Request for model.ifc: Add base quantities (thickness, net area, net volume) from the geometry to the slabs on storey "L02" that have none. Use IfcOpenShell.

First a look at what the model holds.

```python
import ifcopenshell
import ifcopenshell.util.element
import ifcopenshell.util.unit

model = ifcopenshell.open("model.ifc")
print(model.schema)
for unit_type in ("LENGTHUNIT", "AREAUNIT", "VOLUMEUNIT"):
    print(unit_type, ifcopenshell.util.unit.calculate_unit_scale(model, unit_type))
storey = next(s for s in model.by_type("IfcBuildingStorey") if s.Name == "L02")
slabs = [e for e in ifcopenshell.util.element.get_decomposition(storey) if e.is_a("IfcSlab")]
for e in sorted(slabs, key=lambda e: e.id()):
    print(e.id(), e.is_a(), e.Name, list(ifcopenshell.util.element.get_psets(e, qtos_only=True)), sep=" | ")
```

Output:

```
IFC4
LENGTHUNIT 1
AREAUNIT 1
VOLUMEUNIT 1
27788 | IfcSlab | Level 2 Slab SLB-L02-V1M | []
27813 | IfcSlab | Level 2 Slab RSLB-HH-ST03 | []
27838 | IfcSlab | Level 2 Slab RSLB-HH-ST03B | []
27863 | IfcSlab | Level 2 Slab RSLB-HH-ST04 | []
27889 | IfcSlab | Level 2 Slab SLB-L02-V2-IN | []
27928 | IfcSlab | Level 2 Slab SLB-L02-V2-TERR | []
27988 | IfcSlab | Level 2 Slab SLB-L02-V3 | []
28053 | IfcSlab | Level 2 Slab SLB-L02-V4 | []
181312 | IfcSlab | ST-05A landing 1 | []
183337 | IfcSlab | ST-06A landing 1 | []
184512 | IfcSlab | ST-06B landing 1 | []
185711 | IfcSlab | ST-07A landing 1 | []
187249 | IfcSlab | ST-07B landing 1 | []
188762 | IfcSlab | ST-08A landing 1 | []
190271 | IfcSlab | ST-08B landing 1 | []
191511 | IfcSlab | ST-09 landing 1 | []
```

```python
import ifcopenshell
import ifcopenshell.api.pset
import ifcopenshell.geom
import ifcopenshell.util.element
import ifcopenshell.util.shape
import ifcopenshell.util.unit

model = ifcopenshell.open("model.ifc")
unit_scale = ifcopenshell.util.unit.calculate_unit_scale(model)
area_scale = ifcopenshell.util.unit.calculate_unit_scale(model, "AREAUNIT")
volume_scale = ifcopenshell.util.unit.calculate_unit_scale(model, "VOLUMEUNIT")
settings = ifcopenshell.geom.settings()

storey = next(s for s in model.by_type("IfcBuildingStorey") if s.Name == "L02")
slabs = [e for e in ifcopenshell.util.element.get_decomposition(storey) if e.is_a("IfcSlab")]

for e in sorted(slabs, key=lambda e: e.id()):
    if ifcopenshell.util.element.get_psets(e, qtos_only=True, should_inherit=False):
        continue
    # Geometry comes back in metres, in the element's own axes.
    shape = ifcopenshell.geom.create_shape(settings, e)
    values = {
        "Width": ifcopenshell.util.shape.get_z(shape.geometry) / unit_scale,
        "NetArea": ifcopenshell.util.shape.get_footprint_area(shape.geometry) / area_scale,
        "NetVolume": ifcopenshell.util.shape.get_volume(shape.geometry) / volume_scale,
    }
    qto = ifcopenshell.api.pset.add_qto(model, product=e, name="Qto_SlabBaseQuantities")
    ifcopenshell.api.pset.edit_qto(model, qto=qto, properties=values)
    print(e.id(), {k: round(v, 3) for k, v in values.items()})

model.write("model_edited.ifc")
```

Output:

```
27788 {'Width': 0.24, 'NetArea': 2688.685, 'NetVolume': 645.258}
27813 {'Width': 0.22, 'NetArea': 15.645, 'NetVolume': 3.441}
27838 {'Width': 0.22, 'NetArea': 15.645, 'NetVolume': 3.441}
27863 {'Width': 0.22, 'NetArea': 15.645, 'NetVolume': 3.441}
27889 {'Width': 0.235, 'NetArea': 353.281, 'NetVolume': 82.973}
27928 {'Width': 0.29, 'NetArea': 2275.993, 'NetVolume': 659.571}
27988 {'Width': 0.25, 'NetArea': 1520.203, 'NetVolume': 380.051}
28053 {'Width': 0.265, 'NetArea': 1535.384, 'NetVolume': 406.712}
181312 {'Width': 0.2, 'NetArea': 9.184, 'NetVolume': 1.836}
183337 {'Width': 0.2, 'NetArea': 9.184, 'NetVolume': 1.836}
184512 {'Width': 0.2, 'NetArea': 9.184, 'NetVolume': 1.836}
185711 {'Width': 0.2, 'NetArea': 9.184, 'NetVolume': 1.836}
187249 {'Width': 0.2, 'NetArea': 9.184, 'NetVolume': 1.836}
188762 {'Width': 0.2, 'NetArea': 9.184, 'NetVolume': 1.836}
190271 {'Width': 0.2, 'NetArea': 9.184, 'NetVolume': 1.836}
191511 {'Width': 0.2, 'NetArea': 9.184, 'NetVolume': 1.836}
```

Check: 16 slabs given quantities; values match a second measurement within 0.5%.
